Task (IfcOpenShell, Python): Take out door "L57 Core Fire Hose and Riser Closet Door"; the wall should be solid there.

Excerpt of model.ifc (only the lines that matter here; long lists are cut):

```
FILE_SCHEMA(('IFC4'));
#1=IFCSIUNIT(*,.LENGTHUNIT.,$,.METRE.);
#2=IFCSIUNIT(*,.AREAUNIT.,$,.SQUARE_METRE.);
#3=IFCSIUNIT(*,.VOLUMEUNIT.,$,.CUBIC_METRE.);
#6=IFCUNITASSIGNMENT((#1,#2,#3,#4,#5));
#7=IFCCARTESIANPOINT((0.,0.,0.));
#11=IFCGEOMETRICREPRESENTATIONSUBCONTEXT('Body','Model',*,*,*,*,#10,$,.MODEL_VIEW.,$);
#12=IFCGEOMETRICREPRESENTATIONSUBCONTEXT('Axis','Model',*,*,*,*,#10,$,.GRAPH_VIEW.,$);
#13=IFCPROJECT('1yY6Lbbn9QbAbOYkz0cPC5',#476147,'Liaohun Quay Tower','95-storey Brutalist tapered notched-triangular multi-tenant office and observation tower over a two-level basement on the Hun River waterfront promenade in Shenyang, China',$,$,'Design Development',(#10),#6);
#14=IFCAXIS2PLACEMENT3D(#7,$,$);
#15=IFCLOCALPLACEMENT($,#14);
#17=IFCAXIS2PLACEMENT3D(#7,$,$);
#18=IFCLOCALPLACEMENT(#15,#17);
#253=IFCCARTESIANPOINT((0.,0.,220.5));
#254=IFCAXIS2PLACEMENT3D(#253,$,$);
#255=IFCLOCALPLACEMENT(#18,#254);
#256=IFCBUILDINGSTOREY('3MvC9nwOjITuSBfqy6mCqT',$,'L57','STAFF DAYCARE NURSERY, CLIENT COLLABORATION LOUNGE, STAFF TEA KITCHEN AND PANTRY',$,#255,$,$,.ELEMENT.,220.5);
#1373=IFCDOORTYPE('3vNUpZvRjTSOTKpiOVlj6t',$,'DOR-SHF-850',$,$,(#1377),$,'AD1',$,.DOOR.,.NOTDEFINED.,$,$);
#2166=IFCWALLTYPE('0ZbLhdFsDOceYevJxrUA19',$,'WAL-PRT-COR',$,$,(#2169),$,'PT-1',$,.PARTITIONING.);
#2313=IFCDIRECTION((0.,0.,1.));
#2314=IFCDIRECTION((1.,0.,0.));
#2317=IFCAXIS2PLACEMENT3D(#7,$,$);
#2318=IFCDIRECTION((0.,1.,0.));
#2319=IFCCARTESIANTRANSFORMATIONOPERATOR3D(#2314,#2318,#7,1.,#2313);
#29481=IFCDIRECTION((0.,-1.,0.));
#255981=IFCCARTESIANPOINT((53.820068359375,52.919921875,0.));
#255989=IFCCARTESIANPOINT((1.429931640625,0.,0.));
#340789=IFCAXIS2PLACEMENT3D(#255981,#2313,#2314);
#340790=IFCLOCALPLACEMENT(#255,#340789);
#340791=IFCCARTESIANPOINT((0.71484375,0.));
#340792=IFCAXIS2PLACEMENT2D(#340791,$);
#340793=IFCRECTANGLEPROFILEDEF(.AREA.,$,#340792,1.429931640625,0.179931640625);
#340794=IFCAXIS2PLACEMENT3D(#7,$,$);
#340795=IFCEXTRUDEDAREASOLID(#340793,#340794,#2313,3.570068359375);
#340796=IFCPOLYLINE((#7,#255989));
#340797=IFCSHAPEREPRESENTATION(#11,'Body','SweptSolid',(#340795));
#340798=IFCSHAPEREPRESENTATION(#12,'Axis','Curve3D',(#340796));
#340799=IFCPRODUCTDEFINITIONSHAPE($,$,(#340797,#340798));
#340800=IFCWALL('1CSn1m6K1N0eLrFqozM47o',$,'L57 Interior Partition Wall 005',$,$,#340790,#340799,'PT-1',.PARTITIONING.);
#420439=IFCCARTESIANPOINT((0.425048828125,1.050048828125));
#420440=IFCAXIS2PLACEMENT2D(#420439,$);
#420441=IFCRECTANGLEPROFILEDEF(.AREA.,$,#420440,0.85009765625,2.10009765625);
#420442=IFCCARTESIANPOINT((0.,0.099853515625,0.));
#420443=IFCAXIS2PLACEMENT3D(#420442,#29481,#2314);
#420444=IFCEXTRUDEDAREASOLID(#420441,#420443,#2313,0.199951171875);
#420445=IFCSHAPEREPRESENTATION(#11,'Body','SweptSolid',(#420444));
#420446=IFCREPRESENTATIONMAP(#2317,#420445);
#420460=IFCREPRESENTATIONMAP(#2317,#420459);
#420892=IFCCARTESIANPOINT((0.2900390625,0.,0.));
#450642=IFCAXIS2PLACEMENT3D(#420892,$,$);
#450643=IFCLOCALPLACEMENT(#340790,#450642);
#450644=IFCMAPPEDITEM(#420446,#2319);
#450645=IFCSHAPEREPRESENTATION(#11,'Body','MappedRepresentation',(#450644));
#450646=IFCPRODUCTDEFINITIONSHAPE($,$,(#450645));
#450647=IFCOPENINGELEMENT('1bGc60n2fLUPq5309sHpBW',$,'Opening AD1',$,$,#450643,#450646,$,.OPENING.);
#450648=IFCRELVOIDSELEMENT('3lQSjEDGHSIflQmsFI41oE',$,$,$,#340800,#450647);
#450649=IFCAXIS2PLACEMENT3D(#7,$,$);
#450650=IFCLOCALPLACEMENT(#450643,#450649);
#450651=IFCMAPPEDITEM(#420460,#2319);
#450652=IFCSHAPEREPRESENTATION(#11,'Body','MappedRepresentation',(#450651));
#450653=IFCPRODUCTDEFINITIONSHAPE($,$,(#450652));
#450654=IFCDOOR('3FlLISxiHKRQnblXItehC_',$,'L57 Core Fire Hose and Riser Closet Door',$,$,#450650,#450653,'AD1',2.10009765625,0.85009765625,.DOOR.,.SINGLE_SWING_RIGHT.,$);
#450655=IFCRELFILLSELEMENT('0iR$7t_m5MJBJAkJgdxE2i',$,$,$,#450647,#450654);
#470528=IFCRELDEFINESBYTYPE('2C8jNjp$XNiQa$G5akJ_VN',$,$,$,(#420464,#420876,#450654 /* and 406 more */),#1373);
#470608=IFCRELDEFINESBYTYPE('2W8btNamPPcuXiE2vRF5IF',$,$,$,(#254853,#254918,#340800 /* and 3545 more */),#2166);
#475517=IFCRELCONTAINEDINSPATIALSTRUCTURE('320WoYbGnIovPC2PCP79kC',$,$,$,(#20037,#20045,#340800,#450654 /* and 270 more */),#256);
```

```python
import ifcopenshell
import ifcopenshell.api.feature
import ifcopenshell.api.root
import ifcopenshell.geom
import ifcopenshell.util.shape

model = ifcopenshell.open("model.ifc")
settings = ifcopenshell.geom.settings()


def volume(element):
    """Net volume in cubic metres, openings subtracted."""
    shape = ifcopenshell.geom.create_shape(settings, element)
    return ifcopenshell.util.shape.get_volume(shape.geometry)


door = model.by_guid("3FlLISxiHKRQnblXItehC_")
opening = door.FillsVoids[0].RelatingOpeningElement
wall = opening.VoidsElements[0].RelatingBuildingElement
before = volume(wall)

ifcopenshell.api.root.remove_product(model, product=door)
ifcopenshell.api.feature.remove_feature(model, feature=opening)

after = volume(wall)

print(f"wall volume {before:.3f} -> {after:.3f} m3")

model.write("model_edited.ifc")
```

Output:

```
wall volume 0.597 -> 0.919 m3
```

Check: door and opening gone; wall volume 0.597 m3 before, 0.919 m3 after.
